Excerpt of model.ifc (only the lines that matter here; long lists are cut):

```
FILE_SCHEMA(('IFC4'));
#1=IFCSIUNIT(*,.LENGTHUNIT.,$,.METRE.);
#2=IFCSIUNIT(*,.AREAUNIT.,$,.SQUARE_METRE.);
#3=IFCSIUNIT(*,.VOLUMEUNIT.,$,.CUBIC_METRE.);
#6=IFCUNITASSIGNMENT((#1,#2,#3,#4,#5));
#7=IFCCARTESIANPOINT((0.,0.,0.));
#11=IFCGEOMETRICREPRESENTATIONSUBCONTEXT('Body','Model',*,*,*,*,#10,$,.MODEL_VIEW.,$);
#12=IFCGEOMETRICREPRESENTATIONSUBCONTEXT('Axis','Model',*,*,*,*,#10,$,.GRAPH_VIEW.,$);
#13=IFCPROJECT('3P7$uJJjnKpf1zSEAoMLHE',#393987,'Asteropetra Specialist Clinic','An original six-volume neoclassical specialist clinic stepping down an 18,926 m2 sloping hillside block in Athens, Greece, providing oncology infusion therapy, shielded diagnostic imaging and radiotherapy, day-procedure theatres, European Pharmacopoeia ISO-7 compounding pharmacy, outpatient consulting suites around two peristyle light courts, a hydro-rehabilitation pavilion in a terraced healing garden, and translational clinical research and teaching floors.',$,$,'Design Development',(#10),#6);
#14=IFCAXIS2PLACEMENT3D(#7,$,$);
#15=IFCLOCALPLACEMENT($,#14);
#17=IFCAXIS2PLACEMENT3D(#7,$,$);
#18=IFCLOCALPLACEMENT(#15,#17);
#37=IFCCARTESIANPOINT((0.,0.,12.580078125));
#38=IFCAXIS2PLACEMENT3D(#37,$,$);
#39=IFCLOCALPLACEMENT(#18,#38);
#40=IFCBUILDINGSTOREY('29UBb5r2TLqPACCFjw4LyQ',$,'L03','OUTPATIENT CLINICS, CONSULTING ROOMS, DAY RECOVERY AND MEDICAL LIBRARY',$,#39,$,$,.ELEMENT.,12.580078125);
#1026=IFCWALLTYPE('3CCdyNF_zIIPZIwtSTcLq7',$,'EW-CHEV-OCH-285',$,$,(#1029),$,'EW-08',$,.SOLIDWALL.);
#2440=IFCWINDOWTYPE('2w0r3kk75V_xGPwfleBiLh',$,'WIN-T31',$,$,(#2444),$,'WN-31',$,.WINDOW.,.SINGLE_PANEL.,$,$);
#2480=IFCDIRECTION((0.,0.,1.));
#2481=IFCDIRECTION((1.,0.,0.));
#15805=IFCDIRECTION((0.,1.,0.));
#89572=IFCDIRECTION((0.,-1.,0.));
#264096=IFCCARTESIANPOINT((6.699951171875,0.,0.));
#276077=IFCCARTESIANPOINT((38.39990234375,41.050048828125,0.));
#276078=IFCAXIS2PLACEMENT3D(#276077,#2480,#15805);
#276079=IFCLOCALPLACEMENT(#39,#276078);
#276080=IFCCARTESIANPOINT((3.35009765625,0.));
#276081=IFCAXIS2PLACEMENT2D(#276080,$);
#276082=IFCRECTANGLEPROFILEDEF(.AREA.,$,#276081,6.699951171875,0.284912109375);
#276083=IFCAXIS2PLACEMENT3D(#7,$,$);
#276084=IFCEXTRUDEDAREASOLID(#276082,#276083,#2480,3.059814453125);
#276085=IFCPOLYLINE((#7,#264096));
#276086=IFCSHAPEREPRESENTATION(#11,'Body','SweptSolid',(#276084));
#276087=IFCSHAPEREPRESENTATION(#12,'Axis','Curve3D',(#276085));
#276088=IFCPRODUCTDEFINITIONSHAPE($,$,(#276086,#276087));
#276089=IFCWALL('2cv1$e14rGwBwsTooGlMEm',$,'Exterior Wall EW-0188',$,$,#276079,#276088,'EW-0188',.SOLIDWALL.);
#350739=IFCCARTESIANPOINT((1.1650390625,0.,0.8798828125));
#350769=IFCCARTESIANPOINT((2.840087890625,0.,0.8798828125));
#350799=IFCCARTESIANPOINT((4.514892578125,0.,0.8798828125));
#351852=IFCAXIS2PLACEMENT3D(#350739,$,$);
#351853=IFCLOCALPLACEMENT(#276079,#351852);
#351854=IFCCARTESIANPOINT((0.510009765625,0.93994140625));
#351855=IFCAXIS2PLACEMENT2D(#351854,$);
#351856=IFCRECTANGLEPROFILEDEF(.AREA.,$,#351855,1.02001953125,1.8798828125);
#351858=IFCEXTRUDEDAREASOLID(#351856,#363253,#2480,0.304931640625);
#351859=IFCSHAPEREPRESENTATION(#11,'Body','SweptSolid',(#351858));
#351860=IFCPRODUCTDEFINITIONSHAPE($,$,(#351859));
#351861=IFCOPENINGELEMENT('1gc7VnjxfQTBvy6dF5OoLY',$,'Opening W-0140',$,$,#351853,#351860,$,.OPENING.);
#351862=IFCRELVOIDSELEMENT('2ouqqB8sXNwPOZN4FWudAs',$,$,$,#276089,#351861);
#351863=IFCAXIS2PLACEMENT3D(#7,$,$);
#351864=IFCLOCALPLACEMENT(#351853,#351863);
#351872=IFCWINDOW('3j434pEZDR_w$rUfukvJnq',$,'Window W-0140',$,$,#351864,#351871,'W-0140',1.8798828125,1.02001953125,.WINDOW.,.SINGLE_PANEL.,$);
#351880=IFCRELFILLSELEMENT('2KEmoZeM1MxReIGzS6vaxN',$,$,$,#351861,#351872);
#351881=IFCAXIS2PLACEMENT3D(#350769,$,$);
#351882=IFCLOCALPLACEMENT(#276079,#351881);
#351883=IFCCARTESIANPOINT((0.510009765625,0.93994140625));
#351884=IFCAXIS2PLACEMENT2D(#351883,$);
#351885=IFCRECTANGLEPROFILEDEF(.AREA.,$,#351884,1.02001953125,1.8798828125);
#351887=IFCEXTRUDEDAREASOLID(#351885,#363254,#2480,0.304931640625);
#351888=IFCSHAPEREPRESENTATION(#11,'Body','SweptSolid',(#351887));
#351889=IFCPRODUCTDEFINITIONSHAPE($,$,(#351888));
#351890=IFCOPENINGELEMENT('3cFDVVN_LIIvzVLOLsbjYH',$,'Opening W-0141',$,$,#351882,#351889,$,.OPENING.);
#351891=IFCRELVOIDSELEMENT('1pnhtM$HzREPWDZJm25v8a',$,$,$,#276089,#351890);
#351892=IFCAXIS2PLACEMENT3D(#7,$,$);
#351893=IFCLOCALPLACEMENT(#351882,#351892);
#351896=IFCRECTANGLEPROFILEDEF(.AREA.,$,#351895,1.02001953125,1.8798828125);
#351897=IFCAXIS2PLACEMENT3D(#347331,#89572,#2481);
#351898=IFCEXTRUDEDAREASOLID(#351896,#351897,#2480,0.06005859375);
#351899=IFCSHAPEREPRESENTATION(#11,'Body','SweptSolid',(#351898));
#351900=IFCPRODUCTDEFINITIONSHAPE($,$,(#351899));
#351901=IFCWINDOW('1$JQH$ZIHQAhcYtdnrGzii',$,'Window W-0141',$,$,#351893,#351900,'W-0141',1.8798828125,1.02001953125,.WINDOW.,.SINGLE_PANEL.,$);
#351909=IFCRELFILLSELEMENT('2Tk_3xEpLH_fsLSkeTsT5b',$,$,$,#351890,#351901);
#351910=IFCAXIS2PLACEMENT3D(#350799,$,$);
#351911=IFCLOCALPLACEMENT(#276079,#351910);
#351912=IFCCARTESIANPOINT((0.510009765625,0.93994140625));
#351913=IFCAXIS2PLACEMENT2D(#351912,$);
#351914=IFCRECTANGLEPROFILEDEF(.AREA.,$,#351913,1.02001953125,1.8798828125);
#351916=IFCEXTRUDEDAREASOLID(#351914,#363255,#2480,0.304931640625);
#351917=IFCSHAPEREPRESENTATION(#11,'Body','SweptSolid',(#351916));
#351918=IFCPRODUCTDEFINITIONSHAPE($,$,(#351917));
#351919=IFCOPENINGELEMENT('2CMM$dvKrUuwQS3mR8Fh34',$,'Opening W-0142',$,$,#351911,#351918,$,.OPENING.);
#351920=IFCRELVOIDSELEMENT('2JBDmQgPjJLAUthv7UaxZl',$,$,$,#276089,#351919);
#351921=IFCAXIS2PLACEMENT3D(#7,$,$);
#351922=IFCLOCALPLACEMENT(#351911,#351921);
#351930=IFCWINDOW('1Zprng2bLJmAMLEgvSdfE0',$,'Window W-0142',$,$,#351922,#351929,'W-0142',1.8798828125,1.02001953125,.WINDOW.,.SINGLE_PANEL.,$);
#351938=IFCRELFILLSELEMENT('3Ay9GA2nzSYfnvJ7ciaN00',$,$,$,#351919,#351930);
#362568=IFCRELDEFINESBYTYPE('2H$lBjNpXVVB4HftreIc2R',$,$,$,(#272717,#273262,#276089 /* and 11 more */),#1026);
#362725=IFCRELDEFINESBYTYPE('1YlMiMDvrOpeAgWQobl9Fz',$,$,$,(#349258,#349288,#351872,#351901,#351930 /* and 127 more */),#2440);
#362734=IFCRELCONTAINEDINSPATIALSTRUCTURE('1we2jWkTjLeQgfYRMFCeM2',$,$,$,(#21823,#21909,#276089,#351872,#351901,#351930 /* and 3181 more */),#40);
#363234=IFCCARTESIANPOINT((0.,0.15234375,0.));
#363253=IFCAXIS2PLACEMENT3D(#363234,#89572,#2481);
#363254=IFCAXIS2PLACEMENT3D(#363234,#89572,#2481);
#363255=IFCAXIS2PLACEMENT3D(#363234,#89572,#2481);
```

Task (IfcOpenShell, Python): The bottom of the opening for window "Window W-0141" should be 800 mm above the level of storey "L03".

```python
import numpy as np
import ifcopenshell
import ifcopenshell.api.geometry
import ifcopenshell.geom
import ifcopenshell.util.element
import ifcopenshell.util.placement
import ifcopenshell.util.shape
import ifcopenshell.util.unit

model = ifcopenshell.open("model.ifc")
unit_scale = ifcopenshell.util.unit.calculate_unit_scale(model)

window = model.by_guid("1$JQH$ZIHQAhcYtdnrGzii")
opening = window.FillsVoids[0].RelatingOpeningElement
storey = ifcopenshell.util.element.get_container(window, ifc_class="IfcBuildingStorey")
level = ifcopenshell.util.placement.get_local_placement(storey.ObjectPlacement)[2, 3]

# The opening's origin need not be at the sill, so measure its lowest point.
shape = ifcopenshell.geom.create_shape(ifcopenshell.geom.settings(), opening)
bottom = ifcopenshell.util.shape.get_shape_bottom_elevation(shape, shape.geometry) / unit_scale
dz = level + 0.8 / unit_scale - bottom

shift = np.array([0.0, 0.0, dz])
# The window is placed relative to its opening, so it follows when the opening moves.
matrix = ifcopenshell.util.placement.get_local_placement(opening.ObjectPlacement)
matrix[:3, 3] += shift
ifcopenshell.api.geometry.edit_object_placement(
    model, product=opening, matrix=matrix, is_si=False, should_transform_children=True
)

print(f"moved by {dz * unit_scale:+.3f} m")

model.write("model_rev.ifc")
```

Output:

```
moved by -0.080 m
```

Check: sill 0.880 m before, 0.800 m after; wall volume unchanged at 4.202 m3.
